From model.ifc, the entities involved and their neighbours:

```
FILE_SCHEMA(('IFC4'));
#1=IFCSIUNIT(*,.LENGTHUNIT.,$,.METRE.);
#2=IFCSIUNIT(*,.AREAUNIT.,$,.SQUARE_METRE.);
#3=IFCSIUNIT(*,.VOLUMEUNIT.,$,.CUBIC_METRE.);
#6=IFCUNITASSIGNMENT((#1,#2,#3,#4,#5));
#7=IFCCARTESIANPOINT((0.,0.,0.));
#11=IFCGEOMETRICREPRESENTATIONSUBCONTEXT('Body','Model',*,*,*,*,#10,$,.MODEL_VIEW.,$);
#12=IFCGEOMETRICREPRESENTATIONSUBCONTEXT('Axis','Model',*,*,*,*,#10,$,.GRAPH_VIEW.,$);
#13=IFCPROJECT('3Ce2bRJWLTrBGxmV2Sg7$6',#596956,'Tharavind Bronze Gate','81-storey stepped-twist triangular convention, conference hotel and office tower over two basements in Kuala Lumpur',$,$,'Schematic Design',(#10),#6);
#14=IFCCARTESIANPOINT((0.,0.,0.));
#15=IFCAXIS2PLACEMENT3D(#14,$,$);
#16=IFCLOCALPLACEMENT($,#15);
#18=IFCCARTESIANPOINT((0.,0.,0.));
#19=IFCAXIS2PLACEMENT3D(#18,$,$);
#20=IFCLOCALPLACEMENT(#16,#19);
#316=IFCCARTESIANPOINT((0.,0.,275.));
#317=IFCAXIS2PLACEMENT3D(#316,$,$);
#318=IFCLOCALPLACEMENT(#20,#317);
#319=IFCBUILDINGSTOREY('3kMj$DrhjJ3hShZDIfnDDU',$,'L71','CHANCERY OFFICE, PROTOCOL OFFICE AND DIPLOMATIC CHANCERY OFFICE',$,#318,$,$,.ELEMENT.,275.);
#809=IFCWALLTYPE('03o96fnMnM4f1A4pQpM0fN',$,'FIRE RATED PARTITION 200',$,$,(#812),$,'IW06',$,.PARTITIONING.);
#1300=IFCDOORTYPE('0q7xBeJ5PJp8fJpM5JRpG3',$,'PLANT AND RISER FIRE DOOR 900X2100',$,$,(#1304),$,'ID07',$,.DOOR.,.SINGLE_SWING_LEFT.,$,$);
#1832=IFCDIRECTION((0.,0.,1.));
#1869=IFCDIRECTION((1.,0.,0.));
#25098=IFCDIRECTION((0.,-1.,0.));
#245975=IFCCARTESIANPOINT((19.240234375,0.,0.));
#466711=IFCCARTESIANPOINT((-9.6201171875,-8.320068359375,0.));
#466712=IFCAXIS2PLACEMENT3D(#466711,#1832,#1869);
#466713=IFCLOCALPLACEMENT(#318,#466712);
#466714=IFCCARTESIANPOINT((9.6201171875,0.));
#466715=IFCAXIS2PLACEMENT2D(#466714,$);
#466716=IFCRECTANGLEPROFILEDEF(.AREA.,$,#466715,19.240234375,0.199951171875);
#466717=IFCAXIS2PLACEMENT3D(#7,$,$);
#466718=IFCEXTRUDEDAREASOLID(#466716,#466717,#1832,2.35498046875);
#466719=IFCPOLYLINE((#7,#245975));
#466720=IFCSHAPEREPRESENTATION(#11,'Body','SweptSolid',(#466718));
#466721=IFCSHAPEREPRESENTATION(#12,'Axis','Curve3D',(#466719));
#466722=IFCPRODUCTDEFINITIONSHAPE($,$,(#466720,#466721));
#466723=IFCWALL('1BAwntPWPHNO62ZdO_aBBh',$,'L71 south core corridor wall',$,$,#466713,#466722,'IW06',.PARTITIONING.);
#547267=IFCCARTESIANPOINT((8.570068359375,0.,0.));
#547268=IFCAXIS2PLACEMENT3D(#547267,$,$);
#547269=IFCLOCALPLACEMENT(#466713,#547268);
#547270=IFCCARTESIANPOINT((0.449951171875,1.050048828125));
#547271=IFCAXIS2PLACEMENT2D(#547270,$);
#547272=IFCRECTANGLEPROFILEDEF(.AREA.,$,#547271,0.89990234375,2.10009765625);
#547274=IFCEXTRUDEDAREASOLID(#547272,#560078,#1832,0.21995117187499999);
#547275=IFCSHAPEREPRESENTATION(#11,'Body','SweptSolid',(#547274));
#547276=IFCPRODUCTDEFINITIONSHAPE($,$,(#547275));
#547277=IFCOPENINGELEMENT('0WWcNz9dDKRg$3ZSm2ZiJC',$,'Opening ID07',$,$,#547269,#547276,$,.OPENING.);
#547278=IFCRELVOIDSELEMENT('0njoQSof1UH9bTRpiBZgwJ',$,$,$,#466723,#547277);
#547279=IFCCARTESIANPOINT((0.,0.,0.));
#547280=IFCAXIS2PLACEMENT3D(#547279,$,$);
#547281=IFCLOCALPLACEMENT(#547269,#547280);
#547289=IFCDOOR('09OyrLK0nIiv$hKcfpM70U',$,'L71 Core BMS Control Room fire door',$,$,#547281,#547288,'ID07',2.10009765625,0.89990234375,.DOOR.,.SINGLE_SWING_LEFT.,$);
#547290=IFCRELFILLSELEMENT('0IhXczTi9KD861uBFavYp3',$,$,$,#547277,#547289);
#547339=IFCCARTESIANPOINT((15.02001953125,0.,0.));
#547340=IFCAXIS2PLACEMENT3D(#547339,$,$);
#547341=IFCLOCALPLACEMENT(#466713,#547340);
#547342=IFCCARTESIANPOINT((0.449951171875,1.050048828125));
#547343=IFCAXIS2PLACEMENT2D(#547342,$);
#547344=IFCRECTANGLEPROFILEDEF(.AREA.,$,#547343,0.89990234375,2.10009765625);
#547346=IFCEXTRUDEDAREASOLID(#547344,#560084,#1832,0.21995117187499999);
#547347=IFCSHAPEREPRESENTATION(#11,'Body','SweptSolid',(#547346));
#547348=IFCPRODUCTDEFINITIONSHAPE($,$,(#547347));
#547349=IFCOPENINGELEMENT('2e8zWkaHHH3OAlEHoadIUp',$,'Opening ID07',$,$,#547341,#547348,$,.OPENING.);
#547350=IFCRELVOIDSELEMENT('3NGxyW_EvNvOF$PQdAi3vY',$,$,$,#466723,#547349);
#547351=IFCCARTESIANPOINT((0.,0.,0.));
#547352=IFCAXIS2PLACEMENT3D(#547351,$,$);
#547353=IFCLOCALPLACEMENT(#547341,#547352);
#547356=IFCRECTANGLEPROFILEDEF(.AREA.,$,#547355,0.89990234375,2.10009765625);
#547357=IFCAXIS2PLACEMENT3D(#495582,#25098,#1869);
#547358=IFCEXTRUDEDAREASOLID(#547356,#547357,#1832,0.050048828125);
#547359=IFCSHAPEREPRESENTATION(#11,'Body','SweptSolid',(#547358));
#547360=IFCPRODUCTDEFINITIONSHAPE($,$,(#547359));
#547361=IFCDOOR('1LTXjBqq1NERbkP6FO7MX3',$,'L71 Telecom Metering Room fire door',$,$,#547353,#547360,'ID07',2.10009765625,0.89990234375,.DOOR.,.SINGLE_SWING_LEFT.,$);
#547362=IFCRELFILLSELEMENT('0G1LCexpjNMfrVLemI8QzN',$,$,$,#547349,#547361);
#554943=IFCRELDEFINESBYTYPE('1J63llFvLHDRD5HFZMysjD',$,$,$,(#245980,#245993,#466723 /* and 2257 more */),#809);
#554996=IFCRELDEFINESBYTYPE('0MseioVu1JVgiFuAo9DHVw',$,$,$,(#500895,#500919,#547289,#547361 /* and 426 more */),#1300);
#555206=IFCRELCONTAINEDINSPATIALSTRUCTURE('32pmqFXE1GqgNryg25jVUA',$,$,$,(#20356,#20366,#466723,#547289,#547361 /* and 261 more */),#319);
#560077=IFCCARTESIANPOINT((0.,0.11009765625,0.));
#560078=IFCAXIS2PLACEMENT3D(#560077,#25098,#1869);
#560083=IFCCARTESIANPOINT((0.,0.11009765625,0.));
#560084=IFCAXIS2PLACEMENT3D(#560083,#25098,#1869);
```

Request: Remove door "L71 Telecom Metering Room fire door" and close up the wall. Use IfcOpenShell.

```python
import ifcopenshell
import ifcopenshell.api.feature
import ifcopenshell.api.root
import ifcopenshell.geom
import ifcopenshell.util.shape

model = ifcopenshell.open("model.ifc")
settings = ifcopenshell.geom.settings()


def volume(element):
    """Net volume in cubic metres, openings subtracted."""
    shape = ifcopenshell.geom.create_shape(settings, element)
    return ifcopenshell.util.shape.get_volume(shape.geometry)


door = model.by_guid("1LTXjBqq1NERbkP6FO7MX3")
opening = door.FillsVoids[0].RelatingOpeningElement
wall = opening.VoidsElements[0].RelatingBuildingElement
before = volume(wall)

ifcopenshell.api.root.remove_product(model, product=door)
ifcopenshell.api.feature.remove_feature(model, feature=opening)

after = volume(wall)

print(f"wall volume {before:.3f} -> {after:.3f} m3")

model.write("model_updated.ifc")
```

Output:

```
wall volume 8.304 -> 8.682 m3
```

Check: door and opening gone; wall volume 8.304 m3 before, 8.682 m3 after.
